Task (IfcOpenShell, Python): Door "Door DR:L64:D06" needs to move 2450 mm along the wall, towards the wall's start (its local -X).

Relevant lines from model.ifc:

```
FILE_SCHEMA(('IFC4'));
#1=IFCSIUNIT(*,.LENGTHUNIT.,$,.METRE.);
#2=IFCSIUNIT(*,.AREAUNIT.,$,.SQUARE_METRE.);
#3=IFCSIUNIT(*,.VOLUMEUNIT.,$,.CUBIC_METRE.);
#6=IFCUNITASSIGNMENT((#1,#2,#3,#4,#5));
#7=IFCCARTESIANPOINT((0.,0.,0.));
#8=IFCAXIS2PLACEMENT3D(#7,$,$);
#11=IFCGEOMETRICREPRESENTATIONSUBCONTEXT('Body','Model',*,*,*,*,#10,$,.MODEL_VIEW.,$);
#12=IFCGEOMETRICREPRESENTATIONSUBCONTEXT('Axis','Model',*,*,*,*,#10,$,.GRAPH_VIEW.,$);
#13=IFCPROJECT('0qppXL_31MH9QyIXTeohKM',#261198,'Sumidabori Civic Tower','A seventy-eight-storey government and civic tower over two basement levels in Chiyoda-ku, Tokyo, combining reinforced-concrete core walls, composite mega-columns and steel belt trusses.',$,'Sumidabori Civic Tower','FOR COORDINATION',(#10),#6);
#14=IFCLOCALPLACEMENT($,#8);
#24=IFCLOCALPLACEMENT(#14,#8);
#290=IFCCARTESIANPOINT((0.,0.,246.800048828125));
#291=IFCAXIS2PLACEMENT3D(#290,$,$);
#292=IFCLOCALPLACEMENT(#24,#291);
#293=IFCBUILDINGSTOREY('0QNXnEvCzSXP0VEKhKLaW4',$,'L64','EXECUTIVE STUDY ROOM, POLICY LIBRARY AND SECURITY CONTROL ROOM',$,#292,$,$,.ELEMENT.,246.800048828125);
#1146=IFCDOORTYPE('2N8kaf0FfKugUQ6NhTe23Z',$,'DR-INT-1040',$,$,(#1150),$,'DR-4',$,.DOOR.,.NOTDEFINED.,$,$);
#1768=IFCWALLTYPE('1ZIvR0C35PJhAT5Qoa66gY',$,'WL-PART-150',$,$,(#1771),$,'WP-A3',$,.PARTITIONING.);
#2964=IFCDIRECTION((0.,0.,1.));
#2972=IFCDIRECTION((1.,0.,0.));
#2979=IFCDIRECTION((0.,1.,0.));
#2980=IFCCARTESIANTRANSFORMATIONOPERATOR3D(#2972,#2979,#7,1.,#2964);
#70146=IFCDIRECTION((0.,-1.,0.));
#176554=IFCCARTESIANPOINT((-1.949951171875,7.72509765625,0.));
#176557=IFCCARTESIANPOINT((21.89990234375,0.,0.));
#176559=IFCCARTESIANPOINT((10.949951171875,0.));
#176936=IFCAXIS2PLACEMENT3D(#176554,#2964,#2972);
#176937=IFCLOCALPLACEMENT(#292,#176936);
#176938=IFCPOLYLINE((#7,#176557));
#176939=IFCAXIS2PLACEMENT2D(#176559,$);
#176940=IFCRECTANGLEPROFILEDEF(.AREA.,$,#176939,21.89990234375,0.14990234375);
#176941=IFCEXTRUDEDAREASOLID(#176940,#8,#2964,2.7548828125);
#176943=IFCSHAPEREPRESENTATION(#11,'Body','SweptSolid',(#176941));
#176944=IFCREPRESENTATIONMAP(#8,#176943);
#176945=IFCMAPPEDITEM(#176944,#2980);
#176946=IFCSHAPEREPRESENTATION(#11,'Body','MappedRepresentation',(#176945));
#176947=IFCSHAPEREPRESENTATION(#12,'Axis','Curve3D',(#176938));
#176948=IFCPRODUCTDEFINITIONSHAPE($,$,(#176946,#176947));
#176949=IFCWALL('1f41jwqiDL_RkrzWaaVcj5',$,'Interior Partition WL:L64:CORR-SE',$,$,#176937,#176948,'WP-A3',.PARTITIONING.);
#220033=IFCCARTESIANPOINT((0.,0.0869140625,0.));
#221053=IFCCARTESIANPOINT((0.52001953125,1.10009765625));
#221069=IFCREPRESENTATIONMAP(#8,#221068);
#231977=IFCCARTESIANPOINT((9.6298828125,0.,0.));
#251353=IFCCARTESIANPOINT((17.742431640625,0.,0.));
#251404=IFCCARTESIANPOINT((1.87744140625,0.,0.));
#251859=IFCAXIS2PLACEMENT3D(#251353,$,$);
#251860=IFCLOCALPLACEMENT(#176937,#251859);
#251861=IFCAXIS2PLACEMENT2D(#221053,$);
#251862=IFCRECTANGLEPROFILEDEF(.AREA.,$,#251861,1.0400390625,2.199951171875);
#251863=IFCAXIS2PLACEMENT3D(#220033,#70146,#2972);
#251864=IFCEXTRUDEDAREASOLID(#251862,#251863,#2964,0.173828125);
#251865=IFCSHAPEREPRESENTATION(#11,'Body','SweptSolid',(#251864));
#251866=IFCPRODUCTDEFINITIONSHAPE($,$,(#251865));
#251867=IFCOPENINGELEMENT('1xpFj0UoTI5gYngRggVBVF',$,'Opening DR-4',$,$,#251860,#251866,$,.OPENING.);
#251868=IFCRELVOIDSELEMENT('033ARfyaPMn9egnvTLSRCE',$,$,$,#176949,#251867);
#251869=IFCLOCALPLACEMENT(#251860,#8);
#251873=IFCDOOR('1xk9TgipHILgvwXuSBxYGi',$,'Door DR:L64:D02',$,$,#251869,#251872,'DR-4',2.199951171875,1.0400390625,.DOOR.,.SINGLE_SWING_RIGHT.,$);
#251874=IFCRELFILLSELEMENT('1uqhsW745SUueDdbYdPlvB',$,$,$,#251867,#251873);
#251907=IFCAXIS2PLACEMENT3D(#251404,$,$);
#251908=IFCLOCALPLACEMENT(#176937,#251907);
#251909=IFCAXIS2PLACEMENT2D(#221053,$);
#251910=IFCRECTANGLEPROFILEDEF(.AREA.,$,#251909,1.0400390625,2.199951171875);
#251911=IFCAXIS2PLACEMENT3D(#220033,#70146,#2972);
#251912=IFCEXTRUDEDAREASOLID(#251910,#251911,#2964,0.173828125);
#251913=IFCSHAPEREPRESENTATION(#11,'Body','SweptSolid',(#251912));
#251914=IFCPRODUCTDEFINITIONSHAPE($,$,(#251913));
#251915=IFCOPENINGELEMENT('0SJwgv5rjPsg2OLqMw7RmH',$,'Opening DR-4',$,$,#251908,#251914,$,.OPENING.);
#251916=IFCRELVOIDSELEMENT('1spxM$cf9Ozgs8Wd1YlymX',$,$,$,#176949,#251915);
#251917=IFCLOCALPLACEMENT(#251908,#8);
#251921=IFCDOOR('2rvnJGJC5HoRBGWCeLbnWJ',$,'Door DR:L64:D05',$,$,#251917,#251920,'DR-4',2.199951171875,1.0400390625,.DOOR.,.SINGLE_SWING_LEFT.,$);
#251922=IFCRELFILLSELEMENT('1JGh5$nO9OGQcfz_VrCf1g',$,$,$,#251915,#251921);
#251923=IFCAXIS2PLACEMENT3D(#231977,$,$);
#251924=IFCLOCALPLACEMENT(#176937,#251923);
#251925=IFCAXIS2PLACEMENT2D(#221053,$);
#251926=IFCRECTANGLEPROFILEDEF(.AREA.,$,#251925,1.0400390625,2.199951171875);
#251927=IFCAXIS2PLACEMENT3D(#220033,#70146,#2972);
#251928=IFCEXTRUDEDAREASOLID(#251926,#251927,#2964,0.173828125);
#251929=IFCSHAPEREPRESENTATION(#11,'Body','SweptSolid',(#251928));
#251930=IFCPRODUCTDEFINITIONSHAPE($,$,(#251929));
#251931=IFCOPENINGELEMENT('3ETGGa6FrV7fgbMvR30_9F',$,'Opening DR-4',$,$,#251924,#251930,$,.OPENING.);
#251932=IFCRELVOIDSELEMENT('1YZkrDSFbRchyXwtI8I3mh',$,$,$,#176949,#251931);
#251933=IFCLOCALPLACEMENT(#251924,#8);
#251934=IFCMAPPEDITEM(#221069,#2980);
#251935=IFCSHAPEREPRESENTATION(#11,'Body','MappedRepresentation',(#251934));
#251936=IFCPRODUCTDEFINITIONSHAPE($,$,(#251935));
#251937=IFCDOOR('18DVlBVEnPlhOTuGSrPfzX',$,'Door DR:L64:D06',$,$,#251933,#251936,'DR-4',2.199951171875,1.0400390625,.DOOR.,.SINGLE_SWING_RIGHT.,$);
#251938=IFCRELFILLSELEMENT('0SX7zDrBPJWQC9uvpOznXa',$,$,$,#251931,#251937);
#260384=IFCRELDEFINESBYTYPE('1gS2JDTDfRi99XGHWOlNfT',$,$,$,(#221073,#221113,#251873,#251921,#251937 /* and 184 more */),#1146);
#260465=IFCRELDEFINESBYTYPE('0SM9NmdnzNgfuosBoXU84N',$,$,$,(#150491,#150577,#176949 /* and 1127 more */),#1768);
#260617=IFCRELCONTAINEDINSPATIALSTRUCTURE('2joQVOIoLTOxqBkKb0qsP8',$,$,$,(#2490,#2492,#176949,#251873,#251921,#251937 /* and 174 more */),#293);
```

```python
import ifcopenshell
import ifcopenshell.api.geometry
import ifcopenshell.util.placement
import ifcopenshell.util.unit

model = ifcopenshell.open("model.ifc")
unit_scale = ifcopenshell.util.unit.calculate_unit_scale(model)

door = model.by_guid("18DVlBVEnPlhOTuGSrPfzX")
opening = door.FillsVoids[0].RelatingOpeningElement
wall = opening.VoidsElements[0].RelatingBuildingElement

wall_matrix = ifcopenshell.util.placement.get_local_placement(wall.ObjectPlacement)
shift = wall_matrix[:3, 0] * -2.45 / unit_scale
before = ifcopenshell.util.placement.get_local_placement(door.ObjectPlacement)[:3, 3].copy()

# The door is placed relative to its opening, so it follows when the opening moves.
matrix = ifcopenshell.util.placement.get_local_placement(opening.ObjectPlacement)
matrix[:3, 3] += shift
ifcopenshell.api.geometry.edit_object_placement(
    model, product=opening, matrix=matrix, is_si=False, should_transform_children=True
)

after = ifcopenshell.util.placement.get_local_placement(door.ObjectPlacement)[:3, 3]
print("door moved by", (after - before).round(3) + 0.0)

model.write("model_updated.ifc")
```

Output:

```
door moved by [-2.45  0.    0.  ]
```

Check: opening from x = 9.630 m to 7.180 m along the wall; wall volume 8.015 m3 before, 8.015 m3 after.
